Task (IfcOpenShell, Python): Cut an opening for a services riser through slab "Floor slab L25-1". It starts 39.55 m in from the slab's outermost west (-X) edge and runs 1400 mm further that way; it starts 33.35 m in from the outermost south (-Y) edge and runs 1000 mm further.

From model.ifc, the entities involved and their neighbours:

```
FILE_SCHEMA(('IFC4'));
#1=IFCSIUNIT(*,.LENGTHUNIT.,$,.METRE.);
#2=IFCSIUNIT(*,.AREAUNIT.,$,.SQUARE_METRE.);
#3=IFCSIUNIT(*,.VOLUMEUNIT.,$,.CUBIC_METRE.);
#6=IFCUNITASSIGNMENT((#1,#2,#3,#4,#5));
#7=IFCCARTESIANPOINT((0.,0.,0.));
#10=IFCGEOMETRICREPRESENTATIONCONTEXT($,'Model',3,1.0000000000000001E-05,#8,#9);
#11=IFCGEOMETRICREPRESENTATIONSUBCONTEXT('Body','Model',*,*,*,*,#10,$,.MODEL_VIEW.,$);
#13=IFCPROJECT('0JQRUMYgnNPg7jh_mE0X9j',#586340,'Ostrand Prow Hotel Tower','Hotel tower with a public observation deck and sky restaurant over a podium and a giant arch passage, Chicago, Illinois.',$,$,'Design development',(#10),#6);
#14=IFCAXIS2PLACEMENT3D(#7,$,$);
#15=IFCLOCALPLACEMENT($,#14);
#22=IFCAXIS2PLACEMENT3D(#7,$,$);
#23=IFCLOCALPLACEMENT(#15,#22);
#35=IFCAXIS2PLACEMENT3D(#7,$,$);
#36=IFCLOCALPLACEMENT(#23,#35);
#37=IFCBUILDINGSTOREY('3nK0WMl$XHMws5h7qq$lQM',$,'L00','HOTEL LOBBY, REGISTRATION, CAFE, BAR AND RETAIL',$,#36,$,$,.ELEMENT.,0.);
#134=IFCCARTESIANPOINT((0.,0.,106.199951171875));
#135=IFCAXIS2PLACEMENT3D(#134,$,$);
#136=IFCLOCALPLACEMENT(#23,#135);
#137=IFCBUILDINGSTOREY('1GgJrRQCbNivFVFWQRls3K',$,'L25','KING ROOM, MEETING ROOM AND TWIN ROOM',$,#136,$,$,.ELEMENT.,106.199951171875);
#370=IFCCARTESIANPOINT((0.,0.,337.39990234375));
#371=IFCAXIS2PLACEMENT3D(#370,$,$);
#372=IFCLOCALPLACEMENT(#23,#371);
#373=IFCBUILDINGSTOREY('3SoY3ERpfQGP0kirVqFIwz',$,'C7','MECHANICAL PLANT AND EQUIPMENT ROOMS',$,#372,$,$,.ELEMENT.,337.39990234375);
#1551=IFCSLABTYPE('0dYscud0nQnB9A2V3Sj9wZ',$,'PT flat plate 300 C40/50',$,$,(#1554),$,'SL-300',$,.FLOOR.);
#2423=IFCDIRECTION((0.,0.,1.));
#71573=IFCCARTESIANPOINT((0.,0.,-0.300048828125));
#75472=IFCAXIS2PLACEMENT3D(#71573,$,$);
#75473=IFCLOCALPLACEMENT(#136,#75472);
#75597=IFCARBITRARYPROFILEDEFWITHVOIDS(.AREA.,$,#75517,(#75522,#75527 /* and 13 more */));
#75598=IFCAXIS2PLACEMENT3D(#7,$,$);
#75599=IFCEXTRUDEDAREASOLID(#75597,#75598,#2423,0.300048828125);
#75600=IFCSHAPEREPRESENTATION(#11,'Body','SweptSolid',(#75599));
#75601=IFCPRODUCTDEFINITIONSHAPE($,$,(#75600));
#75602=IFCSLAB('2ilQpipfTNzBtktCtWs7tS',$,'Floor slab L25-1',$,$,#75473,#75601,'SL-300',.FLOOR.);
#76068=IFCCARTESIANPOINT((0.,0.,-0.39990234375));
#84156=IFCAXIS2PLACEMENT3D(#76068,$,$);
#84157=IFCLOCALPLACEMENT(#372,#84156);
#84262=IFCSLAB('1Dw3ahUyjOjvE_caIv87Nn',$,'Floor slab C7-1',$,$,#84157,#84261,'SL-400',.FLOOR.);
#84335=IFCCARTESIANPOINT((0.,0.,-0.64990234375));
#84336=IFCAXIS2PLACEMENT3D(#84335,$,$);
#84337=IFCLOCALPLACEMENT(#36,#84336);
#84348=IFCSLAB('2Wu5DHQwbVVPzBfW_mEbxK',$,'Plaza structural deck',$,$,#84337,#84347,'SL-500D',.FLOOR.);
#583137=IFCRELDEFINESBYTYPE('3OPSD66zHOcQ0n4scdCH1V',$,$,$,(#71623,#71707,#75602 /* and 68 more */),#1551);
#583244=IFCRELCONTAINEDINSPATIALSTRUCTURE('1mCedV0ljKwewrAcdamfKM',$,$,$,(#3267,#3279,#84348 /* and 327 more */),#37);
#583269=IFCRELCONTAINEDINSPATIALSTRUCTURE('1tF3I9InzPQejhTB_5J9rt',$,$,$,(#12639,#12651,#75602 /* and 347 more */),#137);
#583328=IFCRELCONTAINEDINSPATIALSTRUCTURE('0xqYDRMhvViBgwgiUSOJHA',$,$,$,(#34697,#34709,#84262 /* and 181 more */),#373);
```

```python
import numpy as np
import ifcopenshell
import ifcopenshell.api.feature
import ifcopenshell.api.geometry
import ifcopenshell.api.root
import ifcopenshell.geom
import ifcopenshell.util.placement
import ifcopenshell.util.representation
import ifcopenshell.util.shape
import ifcopenshell.util.unit

model = ifcopenshell.open("model.ifc")
unit_scale = ifcopenshell.util.unit.calculate_unit_scale(model)
settings = ifcopenshell.geom.settings()


def volume(element):
    """Net volume in cubic metres, openings subtracted."""
    shape = ifcopenshell.geom.create_shape(settings, element)
    return ifcopenshell.util.shape.get_volume(shape.geometry)


slab = model.by_id(75602)
before = volume(slab)

# Extent in the slab's own axes, in metres. The edges named are its -X and -Y sides.
slab_shape = ifcopenshell.geom.create_shape(settings, slab)
vertices = ifcopenshell.util.shape.get_vertices(slab_shape.geometry)
x_min, y_min, bottom = vertices.min(axis=0)
top = vertices[:, 2].max()

opening = ifcopenshell.api.root.create_entity(model, ifc_class="IfcOpeningElement", name="Services riser opening", predefined_type="OPENING")
context = ifcopenshell.util.representation.get_context(model, "Model", "Body", "MODEL_VIEW")
width, depth = 1.4, 1
outline = [(0.0, 0.0), (width, 0.0), (width, depth), (0.0, depth), (0.0, 0.0)]
# Overshoot both faces by 50 mm so the cut is clean.
shape = ifcopenshell.api.geometry.add_slab_representation(
    model, context=context, depth=top - bottom + 0.1, polyline=outline
)
ifcopenshell.api.geometry.assign_representation(model, product=opening, representation=shape)

matrix = ifcopenshell.util.placement.get_local_placement(slab.ObjectPlacement)
matrix[:, 3] = matrix @ np.append(np.array([x_min + 39.55, y_min + 33.35, bottom - 0.05]) / unit_scale, 1.0)
ifcopenshell.api.geometry.edit_object_placement(model, product=opening, matrix=matrix, is_si=False)
ifcopenshell.api.feature.add_feature(model, feature=opening, element=slab)

after = volume(slab)

print(f"slab volume {before:.3f} -> {after:.3f} m3")

model.write("model_updated.ifc")
```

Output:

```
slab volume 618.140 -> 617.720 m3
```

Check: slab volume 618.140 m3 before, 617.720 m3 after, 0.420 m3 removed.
